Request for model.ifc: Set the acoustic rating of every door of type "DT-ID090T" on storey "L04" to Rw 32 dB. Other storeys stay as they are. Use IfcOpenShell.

First a look at what the model holds.

```python
import ifcopenshell
import ifcopenshell.util.element

model = ifcopenshell.open("model.ifc")
print(model.schema)
storey = next(s for s in model.by_type("IfcBuildingStorey") if s.Name == "L04")
doors = [e for e in ifcopenshell.util.element.get_decomposition(storey) if e.is_a("IfcDoor")]
seen = {}
for e in doors:
    element_type = ifcopenshell.util.element.get_type(e)
    key = (element_type.Name if element_type != e and element_type else None, ifcopenshell.util.element.get_pset(e, "Pset_DoorCommon", "AcousticRating"))
    seen[key] = seen.get(key, 0) + 1
for (name, value), count in sorted(seen.items(), key=str):
    print(count, "x", name, "|", value)
```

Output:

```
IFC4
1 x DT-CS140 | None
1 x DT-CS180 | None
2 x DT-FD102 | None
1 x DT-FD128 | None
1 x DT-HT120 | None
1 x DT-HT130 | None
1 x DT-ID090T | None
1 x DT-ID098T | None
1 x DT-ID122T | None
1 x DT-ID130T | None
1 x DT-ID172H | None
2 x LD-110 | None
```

```python
import ifcopenshell
import ifcopenshell.api.pset
import ifcopenshell.util.element

model = ifcopenshell.open("model.ifc")

storey = next(s for s in model.by_type("IfcBuildingStorey") if s.Name == "L04")
doors = [e for e in ifcopenshell.util.element.get_decomposition(storey) if e.is_a("IfcDoor")]

count = 0
for e in doors:
    element_type = ifcopenshell.util.element.get_type(e)
    if element_type in (None, e) or element_type.Name != "DT-ID090T":
        continue
    # add_pset returns the element's existing set when there is one.
    pset = ifcopenshell.api.pset.add_pset(model, product=e, name="Pset_DoorCommon")
    ifcopenshell.api.pset.edit_pset(model, pset=pset, properties={"AcousticRating": "Rw 32 dB"})
    count += 1

print(count, "doors updated")

model.write("model_rev.ifc")
```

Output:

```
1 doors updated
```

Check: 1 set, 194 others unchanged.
